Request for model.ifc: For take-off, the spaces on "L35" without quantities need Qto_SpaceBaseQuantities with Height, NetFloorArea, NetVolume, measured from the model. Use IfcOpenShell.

First a look at what the model holds.

```python
import ifcopenshell
import ifcopenshell.util.element
import ifcopenshell.util.unit

model = ifcopenshell.open("model.ifc")
print(model.schema)
for unit_type in ("LENGTHUNIT", "AREAUNIT", "VOLUMEUNIT"):
    print(unit_type, ifcopenshell.util.unit.calculate_unit_scale(model, unit_type))
storey = next(s for s in model.by_type("IfcBuildingStorey") if s.Name == "L35")
spaces = [e for e in ifcopenshell.util.element.get_decomposition(storey) if e.is_a("IfcSpace")]
for e in sorted(spaces, key=lambda e: e.id()):
    print(e.id(), e.is_a(), e.Name, list(ifcopenshell.util.element.get_psets(e, qtos_only=True)), sep=" | ")
```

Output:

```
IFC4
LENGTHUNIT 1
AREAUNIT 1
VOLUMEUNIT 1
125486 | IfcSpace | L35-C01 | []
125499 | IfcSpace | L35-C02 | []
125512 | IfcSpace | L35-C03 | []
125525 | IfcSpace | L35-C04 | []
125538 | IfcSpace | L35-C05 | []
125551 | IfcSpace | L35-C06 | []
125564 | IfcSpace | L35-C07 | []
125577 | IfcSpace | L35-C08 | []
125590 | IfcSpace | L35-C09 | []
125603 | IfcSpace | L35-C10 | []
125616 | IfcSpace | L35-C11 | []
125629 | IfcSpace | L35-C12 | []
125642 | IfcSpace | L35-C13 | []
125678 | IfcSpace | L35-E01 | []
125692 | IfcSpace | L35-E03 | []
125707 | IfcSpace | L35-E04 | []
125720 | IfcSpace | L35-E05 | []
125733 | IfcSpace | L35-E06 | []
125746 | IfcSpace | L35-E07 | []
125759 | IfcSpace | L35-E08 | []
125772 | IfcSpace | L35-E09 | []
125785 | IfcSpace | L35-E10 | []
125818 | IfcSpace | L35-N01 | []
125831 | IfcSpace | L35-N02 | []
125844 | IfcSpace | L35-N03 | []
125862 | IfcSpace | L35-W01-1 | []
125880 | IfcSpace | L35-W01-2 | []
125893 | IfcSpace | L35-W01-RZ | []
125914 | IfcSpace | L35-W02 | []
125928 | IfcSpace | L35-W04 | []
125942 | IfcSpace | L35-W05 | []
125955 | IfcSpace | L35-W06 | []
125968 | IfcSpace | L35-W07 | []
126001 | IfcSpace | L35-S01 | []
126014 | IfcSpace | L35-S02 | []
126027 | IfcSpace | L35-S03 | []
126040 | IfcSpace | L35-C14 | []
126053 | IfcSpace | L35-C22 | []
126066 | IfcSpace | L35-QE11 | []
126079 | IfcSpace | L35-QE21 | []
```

```python
import ifcopenshell
import ifcopenshell.api.pset
import ifcopenshell.geom
import ifcopenshell.util.element
import ifcopenshell.util.shape
import ifcopenshell.util.unit

model = ifcopenshell.open("model.ifc")
unit_scale = ifcopenshell.util.unit.calculate_unit_scale(model)
area_scale = ifcopenshell.util.unit.calculate_unit_scale(model, "AREAUNIT")
volume_scale = ifcopenshell.util.unit.calculate_unit_scale(model, "VOLUMEUNIT")
settings = ifcopenshell.geom.settings()

storey = next(s for s in model.by_type("IfcBuildingStorey") if s.Name == "L35")
spaces = [e for e in ifcopenshell.util.element.get_decomposition(storey) if e.is_a("IfcSpace")]

for e in sorted(spaces, key=lambda e: e.id()):
    if ifcopenshell.util.element.get_psets(e, qtos_only=True, should_inherit=False):
        continue
    # Geometry comes back in metres, in the element's own axes.
    shape = ifcopenshell.geom.create_shape(settings, e)
    values = {
        "Height": ifcopenshell.util.shape.get_z(shape.geometry) / unit_scale,
        "NetFloorArea": ifcopenshell.util.shape.get_footprint_area(shape.geometry) / area_scale,
        "NetVolume": ifcopenshell.util.shape.get_volume(shape.geometry) / volume_scale,
    }
    qto = ifcopenshell.api.pset.add_qto(model, product=e, name="Qto_SpaceBaseQuantities")
    ifcopenshell.api.pset.edit_qto(model, qto=qto, properties=values)
    print(e.id(), {k: round(v, 3) for k, v in values.items()})

model.write("model_updated.ifc")
```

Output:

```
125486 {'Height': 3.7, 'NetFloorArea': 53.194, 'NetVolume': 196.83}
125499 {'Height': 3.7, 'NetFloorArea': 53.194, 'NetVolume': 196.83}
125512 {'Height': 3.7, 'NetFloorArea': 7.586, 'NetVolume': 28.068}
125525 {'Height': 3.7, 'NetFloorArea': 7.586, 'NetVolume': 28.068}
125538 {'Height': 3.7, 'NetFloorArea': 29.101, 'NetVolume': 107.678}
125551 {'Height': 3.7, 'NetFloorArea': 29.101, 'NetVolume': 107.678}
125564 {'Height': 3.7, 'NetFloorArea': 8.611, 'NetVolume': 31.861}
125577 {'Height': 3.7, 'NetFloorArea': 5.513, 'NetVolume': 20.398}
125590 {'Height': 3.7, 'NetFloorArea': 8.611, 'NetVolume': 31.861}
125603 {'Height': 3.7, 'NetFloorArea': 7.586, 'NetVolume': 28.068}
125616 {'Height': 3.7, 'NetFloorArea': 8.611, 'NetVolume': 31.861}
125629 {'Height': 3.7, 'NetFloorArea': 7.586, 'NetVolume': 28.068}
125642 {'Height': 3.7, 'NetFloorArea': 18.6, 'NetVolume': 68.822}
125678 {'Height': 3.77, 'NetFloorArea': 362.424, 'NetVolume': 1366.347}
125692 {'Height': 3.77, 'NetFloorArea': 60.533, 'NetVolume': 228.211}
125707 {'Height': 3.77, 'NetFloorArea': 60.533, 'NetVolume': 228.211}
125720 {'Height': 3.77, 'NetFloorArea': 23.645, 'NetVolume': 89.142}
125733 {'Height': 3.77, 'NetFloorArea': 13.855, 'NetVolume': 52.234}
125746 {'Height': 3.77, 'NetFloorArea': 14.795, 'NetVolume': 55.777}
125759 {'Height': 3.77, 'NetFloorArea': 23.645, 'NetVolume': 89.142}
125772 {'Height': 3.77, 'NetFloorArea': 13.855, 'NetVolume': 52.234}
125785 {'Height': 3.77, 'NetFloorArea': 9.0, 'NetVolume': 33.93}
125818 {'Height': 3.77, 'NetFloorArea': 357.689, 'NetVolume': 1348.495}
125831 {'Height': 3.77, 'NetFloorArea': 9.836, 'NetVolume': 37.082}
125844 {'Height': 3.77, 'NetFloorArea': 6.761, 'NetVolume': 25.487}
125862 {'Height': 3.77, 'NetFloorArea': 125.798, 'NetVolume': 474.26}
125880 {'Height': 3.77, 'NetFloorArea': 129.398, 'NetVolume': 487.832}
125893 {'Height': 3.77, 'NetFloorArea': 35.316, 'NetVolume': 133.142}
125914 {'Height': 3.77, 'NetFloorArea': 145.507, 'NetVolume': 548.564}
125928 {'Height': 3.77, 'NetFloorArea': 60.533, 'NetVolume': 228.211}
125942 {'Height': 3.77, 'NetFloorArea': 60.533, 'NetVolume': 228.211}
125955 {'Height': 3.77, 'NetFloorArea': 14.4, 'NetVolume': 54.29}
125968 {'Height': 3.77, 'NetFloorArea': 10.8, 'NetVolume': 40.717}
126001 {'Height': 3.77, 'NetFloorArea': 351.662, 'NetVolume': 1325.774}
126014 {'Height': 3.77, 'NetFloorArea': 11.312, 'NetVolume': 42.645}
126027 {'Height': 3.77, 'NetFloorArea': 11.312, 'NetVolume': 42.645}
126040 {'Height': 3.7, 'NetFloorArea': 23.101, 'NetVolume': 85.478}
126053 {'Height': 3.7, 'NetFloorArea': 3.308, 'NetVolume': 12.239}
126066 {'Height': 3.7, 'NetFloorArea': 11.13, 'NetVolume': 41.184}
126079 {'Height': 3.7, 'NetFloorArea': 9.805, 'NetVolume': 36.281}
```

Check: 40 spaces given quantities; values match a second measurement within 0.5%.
